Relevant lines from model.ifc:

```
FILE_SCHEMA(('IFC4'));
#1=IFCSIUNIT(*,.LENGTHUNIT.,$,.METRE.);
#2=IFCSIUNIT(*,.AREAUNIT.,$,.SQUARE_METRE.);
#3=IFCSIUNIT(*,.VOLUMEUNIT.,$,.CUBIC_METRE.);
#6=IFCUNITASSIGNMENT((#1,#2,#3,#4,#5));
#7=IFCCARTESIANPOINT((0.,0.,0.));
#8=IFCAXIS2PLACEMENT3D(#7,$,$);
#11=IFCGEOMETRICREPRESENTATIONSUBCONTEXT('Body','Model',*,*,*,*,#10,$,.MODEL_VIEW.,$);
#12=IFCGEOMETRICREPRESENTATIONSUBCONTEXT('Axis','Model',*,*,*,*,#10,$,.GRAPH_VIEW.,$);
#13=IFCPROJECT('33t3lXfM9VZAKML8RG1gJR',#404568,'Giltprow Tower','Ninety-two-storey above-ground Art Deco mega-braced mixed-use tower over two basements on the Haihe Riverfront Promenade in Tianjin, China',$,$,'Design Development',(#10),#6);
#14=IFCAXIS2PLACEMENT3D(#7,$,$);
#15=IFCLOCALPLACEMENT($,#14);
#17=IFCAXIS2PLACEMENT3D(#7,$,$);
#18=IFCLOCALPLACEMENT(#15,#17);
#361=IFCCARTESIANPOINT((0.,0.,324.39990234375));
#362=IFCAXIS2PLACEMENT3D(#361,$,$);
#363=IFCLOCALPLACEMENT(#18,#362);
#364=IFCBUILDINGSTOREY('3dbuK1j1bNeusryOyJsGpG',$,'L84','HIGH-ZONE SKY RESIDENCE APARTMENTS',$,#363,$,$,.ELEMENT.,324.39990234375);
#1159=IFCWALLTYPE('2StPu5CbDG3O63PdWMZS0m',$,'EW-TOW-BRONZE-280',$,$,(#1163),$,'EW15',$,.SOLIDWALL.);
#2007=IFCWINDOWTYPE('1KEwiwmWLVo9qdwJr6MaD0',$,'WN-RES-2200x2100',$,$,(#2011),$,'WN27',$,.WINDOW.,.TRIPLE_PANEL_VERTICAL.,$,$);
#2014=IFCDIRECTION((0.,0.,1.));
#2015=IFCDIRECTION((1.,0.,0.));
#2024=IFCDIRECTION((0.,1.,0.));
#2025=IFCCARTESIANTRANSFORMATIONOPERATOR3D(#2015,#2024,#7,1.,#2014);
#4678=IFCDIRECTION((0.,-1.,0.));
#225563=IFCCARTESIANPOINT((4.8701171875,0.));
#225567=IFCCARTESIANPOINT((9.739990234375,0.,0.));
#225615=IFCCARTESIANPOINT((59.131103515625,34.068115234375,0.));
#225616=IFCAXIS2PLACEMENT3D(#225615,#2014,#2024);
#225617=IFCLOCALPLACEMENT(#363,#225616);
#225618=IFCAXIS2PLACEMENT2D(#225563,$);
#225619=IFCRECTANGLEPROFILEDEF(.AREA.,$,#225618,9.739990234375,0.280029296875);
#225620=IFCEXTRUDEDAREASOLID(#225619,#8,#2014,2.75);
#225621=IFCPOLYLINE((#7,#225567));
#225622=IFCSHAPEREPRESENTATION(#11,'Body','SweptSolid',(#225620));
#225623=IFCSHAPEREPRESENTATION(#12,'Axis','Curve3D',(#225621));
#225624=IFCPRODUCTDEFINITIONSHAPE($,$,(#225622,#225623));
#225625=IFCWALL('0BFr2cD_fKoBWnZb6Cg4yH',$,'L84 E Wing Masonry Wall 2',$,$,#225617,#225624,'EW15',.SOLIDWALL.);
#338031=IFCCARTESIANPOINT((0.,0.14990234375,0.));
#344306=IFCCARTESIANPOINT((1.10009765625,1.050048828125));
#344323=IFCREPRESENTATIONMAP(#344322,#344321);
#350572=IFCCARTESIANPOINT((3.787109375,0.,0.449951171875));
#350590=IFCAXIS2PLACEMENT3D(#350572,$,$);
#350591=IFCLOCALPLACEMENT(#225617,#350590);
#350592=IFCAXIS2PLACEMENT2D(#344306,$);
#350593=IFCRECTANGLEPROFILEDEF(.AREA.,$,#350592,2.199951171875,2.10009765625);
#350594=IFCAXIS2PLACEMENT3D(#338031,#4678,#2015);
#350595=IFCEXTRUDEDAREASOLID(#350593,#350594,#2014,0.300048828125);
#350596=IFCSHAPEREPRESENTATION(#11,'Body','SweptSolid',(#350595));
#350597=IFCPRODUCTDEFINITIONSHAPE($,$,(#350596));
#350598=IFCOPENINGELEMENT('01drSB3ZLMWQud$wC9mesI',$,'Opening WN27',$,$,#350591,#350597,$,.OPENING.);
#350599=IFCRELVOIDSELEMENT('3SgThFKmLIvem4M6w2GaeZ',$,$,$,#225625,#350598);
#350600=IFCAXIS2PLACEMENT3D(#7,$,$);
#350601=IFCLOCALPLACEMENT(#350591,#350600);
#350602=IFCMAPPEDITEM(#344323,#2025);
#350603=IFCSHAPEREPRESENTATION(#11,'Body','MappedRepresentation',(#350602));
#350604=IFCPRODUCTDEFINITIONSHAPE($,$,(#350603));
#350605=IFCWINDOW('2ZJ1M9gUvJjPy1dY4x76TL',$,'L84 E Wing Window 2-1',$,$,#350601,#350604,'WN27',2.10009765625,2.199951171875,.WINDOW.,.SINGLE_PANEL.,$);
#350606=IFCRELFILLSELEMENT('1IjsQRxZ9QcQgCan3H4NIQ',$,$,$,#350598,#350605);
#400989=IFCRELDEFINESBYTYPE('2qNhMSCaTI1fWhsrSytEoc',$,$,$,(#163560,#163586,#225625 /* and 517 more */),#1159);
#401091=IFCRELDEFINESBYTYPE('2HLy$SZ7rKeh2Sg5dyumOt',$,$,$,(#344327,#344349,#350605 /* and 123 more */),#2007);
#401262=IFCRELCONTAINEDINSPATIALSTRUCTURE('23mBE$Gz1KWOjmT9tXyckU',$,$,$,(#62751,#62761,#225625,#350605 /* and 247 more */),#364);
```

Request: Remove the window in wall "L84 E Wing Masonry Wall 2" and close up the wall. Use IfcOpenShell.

```python
import ifcopenshell
import ifcopenshell.api.feature
import ifcopenshell.api.root
import ifcopenshell.geom
import ifcopenshell.util.shape

model = ifcopenshell.open("model.ifc")
settings = ifcopenshell.geom.settings()


def volume(element):
    """Net volume in cubic metres, openings subtracted."""
    shape = ifcopenshell.geom.create_shape(settings, element)
    return ifcopenshell.util.shape.get_volume(shape.geometry)


window = model.by_id(350605)
opening = window.FillsVoids[0].RelatingOpeningElement
wall = opening.VoidsElements[0].RelatingBuildingElement
before = volume(wall)

ifcopenshell.api.root.remove_product(model, product=window)
ifcopenshell.api.feature.remove_feature(model, feature=opening)

after = volume(wall)

print(f"wall volume {before:.3f} -> {after:.3f} m3")

model.write("model_updated.ifc")
```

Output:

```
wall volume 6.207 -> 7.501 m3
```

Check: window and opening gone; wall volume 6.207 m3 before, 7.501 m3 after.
